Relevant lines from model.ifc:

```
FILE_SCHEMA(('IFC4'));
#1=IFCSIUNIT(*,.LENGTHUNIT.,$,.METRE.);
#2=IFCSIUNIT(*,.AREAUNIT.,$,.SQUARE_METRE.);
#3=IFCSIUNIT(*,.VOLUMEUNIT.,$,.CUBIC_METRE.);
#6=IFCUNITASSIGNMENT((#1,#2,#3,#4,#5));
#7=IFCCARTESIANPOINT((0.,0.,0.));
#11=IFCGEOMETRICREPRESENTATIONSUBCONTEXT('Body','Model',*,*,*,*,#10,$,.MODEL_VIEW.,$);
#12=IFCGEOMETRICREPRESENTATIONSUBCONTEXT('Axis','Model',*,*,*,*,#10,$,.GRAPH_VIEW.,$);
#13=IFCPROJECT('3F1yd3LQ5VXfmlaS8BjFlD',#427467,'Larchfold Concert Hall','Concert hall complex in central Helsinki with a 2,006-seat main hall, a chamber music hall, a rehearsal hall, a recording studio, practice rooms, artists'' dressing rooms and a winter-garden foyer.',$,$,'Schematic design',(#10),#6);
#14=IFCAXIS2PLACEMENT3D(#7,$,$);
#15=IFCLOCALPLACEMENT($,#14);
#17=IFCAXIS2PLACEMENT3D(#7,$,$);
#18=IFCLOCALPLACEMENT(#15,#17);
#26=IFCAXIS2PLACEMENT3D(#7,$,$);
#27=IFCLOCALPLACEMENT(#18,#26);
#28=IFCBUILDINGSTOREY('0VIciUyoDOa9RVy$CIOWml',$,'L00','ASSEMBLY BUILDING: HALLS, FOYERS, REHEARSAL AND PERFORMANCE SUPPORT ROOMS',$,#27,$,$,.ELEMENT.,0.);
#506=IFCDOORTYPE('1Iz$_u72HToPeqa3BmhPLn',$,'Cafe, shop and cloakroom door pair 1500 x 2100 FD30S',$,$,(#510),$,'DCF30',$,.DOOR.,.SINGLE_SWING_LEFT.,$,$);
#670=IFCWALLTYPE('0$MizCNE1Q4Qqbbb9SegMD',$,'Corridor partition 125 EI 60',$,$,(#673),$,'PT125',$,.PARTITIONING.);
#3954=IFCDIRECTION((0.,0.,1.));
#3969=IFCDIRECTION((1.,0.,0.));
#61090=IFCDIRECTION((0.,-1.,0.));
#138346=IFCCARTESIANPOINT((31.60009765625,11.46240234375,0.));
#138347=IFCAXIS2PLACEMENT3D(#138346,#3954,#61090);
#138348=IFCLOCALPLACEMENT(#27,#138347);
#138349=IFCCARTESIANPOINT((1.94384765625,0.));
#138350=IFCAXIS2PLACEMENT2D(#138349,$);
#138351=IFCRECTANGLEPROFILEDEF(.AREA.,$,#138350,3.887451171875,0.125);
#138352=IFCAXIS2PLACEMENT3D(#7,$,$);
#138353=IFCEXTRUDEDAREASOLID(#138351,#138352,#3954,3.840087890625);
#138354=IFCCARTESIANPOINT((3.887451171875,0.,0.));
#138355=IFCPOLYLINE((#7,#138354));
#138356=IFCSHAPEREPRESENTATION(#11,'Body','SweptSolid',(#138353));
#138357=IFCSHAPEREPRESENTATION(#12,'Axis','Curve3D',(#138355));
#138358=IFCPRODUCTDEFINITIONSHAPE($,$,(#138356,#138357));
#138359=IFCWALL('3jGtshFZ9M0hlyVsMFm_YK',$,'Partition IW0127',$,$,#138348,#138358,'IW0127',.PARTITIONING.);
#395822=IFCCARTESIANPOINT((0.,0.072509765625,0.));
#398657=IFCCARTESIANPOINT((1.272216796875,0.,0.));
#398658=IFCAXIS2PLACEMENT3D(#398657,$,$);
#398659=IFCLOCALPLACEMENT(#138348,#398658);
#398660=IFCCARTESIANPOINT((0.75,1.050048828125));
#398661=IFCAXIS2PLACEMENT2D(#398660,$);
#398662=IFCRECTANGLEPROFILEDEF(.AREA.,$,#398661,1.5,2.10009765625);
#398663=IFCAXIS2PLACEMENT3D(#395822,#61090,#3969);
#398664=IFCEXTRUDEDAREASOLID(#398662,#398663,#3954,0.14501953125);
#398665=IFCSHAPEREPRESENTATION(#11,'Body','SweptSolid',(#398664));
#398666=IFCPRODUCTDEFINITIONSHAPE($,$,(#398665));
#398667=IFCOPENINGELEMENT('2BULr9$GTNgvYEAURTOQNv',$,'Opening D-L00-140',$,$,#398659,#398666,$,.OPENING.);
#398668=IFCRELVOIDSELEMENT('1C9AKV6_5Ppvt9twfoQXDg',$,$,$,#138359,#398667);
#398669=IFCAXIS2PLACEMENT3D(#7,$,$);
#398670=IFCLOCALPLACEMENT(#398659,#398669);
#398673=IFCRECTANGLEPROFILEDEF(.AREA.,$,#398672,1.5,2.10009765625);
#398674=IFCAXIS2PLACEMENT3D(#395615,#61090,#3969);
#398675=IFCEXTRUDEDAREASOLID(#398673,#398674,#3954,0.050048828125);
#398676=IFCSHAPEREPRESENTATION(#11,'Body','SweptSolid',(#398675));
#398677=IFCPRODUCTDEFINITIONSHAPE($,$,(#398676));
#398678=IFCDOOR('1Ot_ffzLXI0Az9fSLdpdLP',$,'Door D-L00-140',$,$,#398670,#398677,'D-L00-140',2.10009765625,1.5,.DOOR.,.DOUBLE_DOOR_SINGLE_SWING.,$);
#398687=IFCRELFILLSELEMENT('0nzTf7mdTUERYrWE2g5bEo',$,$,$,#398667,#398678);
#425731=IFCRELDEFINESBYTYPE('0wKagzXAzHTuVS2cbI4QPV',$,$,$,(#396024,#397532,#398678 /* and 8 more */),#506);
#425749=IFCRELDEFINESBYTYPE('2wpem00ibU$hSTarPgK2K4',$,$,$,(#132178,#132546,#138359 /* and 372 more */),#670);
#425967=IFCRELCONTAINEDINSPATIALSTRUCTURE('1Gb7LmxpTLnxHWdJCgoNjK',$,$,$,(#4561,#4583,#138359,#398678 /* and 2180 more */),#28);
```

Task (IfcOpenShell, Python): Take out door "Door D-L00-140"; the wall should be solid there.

```python
import ifcopenshell
import ifcopenshell.api.feature
import ifcopenshell.api.root
import ifcopenshell.geom
import ifcopenshell.util.shape

model = ifcopenshell.open("model.ifc")
settings = ifcopenshell.geom.settings()


def volume(element):
    """Net volume in cubic metres, openings subtracted."""
    shape = ifcopenshell.geom.create_shape(settings, element)
    return ifcopenshell.util.shape.get_volume(shape.geometry)


door = model.by_guid("1Ot_ffzLXI0Az9fSLdpdLP")
opening = door.FillsVoids[0].RelatingOpeningElement
wall = opening.VoidsElements[0].RelatingBuildingElement
before = volume(wall)

ifcopenshell.api.root.remove_product(model, product=door)
ifcopenshell.api.feature.remove_feature(model, feature=opening)

after = volume(wall)

print(f"wall volume {before:.3f} -> {after:.3f} m3")

model.write("model_v2.ifc")
```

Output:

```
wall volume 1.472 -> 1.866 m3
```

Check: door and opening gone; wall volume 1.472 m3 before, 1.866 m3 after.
